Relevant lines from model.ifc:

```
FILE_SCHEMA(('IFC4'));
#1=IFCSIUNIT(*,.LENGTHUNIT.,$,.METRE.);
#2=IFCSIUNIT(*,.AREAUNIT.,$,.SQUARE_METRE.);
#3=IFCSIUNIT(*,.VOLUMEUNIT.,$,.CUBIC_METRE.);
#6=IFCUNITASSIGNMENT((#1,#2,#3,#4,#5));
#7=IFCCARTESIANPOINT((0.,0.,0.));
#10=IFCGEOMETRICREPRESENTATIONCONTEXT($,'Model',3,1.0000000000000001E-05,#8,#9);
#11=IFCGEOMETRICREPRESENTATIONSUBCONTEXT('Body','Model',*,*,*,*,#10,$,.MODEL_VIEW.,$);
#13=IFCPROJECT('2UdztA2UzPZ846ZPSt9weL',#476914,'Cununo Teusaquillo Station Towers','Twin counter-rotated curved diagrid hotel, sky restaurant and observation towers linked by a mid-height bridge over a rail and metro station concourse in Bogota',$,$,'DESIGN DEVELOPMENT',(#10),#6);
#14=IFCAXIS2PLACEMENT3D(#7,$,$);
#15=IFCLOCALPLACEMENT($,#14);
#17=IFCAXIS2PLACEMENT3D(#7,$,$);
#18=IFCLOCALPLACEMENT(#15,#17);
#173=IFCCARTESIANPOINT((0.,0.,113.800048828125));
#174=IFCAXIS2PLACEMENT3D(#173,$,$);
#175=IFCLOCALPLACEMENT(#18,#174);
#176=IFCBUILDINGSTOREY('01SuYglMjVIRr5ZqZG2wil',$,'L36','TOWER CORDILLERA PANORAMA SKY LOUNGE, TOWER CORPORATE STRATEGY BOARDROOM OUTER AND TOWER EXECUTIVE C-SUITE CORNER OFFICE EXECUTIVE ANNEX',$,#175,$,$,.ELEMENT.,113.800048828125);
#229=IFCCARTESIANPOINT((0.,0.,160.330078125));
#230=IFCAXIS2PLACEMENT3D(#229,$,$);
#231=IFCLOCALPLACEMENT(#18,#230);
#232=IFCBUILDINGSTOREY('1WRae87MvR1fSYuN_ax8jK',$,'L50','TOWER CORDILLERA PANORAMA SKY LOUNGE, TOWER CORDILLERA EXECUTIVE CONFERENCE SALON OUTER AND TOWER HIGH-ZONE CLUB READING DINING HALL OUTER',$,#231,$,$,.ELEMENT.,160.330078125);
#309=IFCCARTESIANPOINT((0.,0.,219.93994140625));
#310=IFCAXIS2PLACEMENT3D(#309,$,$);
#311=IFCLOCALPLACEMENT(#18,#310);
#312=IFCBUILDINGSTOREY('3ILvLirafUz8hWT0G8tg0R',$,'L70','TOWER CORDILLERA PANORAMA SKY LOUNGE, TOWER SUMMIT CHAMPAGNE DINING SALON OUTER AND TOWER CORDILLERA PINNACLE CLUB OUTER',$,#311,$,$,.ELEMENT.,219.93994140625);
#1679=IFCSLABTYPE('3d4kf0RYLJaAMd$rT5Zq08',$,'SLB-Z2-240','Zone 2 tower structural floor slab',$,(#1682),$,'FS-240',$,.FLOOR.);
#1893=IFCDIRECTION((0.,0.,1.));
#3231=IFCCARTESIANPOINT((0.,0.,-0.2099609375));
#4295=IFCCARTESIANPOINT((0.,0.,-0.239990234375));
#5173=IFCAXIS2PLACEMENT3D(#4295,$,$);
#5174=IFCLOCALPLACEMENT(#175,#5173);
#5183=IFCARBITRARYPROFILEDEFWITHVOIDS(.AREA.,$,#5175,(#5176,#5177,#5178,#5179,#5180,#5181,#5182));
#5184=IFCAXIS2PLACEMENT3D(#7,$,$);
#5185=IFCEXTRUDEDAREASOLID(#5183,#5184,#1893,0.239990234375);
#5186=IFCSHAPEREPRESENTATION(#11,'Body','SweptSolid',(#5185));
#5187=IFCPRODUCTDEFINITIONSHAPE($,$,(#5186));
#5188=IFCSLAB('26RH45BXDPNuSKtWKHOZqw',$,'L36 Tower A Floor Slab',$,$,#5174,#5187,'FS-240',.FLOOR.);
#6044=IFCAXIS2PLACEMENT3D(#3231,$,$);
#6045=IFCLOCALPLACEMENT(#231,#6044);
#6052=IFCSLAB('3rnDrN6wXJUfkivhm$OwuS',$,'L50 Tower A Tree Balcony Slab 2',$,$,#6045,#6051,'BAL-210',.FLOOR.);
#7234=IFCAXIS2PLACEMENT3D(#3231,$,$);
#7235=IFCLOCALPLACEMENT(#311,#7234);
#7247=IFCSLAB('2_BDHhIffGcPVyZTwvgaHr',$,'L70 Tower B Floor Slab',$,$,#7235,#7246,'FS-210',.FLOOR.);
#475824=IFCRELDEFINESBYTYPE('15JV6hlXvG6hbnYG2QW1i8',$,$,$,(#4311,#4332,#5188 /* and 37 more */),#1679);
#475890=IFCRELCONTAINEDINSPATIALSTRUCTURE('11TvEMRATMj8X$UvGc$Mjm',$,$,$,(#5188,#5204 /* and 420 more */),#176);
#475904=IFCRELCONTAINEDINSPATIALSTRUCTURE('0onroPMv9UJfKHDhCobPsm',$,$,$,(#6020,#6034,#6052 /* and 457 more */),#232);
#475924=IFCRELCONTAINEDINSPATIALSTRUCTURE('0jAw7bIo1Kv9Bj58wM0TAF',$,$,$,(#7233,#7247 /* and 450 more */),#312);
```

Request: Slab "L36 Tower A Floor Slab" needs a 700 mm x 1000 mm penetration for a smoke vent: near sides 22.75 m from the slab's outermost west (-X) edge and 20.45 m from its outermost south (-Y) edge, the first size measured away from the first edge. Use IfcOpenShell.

```python
import numpy as np
import ifcopenshell
import ifcopenshell.api.feature
import ifcopenshell.api.geometry
import ifcopenshell.api.root
import ifcopenshell.geom
import ifcopenshell.util.placement
import ifcopenshell.util.representation
import ifcopenshell.util.shape
import ifcopenshell.util.unit

model = ifcopenshell.open("model.ifc")
unit_scale = ifcopenshell.util.unit.calculate_unit_scale(model)
settings = ifcopenshell.geom.settings()


def volume(element):
    """Net volume in cubic metres, openings subtracted."""
    shape = ifcopenshell.geom.create_shape(settings, element)
    return ifcopenshell.util.shape.get_volume(shape.geometry)


slab = model.by_guid("26RH45BXDPNuSKtWKHOZqw")
before = volume(slab)

# Extent in the slab's own axes, in metres. The edges named are its -X and -Y sides.
slab_shape = ifcopenshell.geom.create_shape(settings, slab)
vertices = ifcopenshell.util.shape.get_vertices(slab_shape.geometry)
x_min, y_min, bottom = vertices.min(axis=0)
top = vertices[:, 2].max()

opening = ifcopenshell.api.root.create_entity(model, ifc_class="IfcOpeningElement", name="Smoke vent opening", predefined_type="OPENING")
context = ifcopenshell.util.representation.get_context(model, "Model", "Body", "MODEL_VIEW")
width, depth = 0.7, 1
outline = [(0.0, 0.0), (width, 0.0), (width, depth), (0.0, depth), (0.0, 0.0)]
# Overshoot both faces by 50 mm so the cut is clean.
shape = ifcopenshell.api.geometry.add_slab_representation(
    model, context=context, depth=top - bottom + 0.1, polyline=outline
)
ifcopenshell.api.geometry.assign_representation(model, product=opening, representation=shape)

matrix = ifcopenshell.util.placement.get_local_placement(slab.ObjectPlacement)
matrix[:, 3] = matrix @ np.append(np.array([x_min + 22.75, y_min + 20.45, bottom - 0.05]) / unit_scale, 1.0)
ifcopenshell.api.geometry.edit_object_placement(model, product=opening, matrix=matrix, is_si=False)
ifcopenshell.api.feature.add_feature(model, feature=opening, element=slab)

after = volume(slab)

print(f"slab volume {before:.3f} -> {after:.3f} m3")

model.write("model_rev.ifc")
```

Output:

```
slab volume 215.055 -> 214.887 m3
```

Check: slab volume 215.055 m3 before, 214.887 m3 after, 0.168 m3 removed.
